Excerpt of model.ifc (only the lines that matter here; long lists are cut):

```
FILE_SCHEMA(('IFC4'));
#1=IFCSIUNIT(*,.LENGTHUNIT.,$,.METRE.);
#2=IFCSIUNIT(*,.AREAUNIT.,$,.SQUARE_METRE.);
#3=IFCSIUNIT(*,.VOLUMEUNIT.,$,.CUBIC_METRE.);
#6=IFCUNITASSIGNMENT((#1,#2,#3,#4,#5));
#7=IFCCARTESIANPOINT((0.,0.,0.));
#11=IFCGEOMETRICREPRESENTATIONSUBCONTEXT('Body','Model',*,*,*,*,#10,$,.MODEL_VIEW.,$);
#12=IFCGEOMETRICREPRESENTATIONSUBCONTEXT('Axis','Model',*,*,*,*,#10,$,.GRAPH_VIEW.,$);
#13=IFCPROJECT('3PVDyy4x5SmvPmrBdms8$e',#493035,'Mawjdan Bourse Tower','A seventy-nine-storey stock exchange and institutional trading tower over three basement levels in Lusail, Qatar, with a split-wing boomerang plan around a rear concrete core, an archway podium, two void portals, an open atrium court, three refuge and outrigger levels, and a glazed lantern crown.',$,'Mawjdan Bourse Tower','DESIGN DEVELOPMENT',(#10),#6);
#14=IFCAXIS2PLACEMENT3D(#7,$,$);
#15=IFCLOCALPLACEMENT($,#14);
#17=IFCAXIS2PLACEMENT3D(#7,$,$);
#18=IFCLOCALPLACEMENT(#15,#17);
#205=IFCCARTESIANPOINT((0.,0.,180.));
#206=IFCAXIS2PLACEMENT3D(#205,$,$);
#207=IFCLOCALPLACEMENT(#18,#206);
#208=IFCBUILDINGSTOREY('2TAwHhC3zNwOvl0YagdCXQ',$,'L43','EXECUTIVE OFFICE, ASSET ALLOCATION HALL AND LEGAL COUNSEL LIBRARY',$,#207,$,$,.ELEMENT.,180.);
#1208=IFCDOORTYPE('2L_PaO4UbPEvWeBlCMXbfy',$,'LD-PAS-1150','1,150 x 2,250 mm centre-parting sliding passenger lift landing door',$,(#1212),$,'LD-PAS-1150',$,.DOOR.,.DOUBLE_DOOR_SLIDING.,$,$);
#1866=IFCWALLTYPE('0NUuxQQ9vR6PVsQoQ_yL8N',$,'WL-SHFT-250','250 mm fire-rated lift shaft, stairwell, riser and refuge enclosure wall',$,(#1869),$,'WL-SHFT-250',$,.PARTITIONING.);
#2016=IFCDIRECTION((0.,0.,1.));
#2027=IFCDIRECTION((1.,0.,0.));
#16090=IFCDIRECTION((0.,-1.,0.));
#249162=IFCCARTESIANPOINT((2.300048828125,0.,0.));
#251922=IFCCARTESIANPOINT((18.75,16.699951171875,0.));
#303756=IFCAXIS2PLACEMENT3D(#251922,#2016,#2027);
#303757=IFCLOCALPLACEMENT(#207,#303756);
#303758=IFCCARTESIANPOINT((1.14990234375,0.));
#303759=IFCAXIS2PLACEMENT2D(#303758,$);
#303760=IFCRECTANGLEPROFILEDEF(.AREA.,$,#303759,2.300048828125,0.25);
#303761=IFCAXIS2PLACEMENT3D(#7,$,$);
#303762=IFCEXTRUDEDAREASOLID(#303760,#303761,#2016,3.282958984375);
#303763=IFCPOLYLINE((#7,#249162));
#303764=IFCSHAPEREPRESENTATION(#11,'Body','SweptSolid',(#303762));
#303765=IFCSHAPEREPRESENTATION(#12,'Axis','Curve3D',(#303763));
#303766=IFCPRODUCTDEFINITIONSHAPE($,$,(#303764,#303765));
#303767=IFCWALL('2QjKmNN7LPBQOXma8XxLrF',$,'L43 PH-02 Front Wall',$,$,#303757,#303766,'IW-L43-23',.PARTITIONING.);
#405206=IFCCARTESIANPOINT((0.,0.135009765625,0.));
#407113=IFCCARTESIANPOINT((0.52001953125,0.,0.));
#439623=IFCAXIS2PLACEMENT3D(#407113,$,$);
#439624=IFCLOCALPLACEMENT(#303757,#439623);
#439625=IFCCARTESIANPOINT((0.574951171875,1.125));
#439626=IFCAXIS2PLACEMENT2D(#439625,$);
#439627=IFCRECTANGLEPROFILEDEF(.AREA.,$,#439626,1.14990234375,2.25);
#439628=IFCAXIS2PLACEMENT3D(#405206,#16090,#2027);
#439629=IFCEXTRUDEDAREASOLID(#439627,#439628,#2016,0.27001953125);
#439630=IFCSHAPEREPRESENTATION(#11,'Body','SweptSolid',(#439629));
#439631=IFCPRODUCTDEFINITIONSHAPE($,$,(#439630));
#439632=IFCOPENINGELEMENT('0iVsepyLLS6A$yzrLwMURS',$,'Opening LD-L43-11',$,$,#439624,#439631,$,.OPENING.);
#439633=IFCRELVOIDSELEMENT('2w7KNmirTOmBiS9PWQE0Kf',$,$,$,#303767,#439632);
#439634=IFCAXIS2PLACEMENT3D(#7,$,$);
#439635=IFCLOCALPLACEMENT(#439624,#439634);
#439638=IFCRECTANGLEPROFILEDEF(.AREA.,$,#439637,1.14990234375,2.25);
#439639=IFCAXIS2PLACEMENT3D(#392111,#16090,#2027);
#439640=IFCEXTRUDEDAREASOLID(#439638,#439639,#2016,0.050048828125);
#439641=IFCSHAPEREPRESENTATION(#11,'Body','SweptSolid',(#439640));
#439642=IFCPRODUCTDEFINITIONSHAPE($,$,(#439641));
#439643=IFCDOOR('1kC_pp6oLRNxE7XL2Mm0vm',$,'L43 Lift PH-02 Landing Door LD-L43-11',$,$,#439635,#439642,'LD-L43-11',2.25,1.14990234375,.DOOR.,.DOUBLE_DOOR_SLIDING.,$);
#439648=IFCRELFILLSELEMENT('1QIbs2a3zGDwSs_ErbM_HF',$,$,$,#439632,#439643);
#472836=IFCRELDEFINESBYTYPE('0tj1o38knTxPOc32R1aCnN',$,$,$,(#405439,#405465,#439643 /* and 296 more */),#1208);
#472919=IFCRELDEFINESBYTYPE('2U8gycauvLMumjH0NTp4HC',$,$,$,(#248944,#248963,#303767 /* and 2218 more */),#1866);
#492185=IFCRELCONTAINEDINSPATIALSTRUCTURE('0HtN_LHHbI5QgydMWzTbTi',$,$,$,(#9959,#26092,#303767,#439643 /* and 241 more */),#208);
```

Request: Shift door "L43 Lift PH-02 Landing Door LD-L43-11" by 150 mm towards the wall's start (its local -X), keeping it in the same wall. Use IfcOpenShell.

```python
import ifcopenshell
import ifcopenshell.api.geometry
import ifcopenshell.util.placement
import ifcopenshell.util.unit

model = ifcopenshell.open("model.ifc")
unit_scale = ifcopenshell.util.unit.calculate_unit_scale(model)

door = model.by_guid("1kC_pp6oLRNxE7XL2Mm0vm")
opening = door.FillsVoids[0].RelatingOpeningElement
wall = opening.VoidsElements[0].RelatingBuildingElement

wall_matrix = ifcopenshell.util.placement.get_local_placement(wall.ObjectPlacement)
shift = wall_matrix[:3, 0] * -0.15 / unit_scale
before = ifcopenshell.util.placement.get_local_placement(door.ObjectPlacement)[:3, 3].copy()

# The door is placed relative to its opening, so it follows when the opening moves.
matrix = ifcopenshell.util.placement.get_local_placement(opening.ObjectPlacement)
matrix[:3, 3] += shift
ifcopenshell.api.geometry.edit_object_placement(
    model, product=opening, matrix=matrix, is_si=False, should_transform_children=True
)

after = ifcopenshell.util.placement.get_local_placement(door.ObjectPlacement)[:3, 3]
print("door moved by", (after - before).round(3) + 0.0)

model.write("model_updated.ifc")
```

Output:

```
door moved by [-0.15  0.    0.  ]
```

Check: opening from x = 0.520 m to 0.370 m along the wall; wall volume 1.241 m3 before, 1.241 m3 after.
